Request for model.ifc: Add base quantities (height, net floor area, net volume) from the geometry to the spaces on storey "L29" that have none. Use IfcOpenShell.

First a look at what the model holds.

```python
import ifcopenshell
import ifcopenshell.util.element
import ifcopenshell.util.unit

model = ifcopenshell.open("model.ifc")
print(model.schema)
for unit_type in ("LENGTHUNIT", "AREAUNIT", "VOLUMEUNIT"):
    print(unit_type, ifcopenshell.util.unit.calculate_unit_scale(model, unit_type))
storey = next(s for s in model.by_type("IfcBuildingStorey") if s.Name == "L29")
spaces = [e for e in ifcopenshell.util.element.get_decomposition(storey) if e.is_a("IfcSpace")]
for e in sorted(spaces, key=lambda e: e.id()):
    print(e.id(), e.is_a(), e.Name, list(ifcopenshell.util.element.get_psets(e, qtos_only=True)), sep=" | ")
```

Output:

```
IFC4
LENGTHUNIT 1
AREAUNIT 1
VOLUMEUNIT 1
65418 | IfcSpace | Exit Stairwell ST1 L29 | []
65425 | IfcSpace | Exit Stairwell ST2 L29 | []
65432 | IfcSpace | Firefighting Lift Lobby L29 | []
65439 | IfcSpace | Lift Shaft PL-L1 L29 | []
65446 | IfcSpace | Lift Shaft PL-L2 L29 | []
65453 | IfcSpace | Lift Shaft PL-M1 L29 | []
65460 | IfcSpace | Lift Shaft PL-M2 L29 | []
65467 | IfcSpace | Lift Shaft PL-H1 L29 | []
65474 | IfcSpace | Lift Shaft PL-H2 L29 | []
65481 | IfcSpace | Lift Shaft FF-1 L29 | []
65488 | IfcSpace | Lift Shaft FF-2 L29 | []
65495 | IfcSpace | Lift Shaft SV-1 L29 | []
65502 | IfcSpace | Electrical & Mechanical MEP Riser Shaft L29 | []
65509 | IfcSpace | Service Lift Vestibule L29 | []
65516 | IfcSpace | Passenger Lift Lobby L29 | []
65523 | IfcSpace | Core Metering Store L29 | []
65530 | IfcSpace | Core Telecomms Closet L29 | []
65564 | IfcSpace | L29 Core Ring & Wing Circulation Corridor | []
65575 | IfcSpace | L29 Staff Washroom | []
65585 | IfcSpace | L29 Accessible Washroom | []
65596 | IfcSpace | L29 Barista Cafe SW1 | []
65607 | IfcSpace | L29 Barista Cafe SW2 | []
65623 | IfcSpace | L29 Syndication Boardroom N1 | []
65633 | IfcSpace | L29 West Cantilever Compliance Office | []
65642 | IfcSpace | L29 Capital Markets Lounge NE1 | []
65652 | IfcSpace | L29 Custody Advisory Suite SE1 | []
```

```python
import ifcopenshell
import ifcopenshell.api.pset
import ifcopenshell.geom
import ifcopenshell.util.element
import ifcopenshell.util.shape
import ifcopenshell.util.unit

model = ifcopenshell.open("model.ifc")
unit_scale = ifcopenshell.util.unit.calculate_unit_scale(model)
area_scale = ifcopenshell.util.unit.calculate_unit_scale(model, "AREAUNIT")
volume_scale = ifcopenshell.util.unit.calculate_unit_scale(model, "VOLUMEUNIT")
settings = ifcopenshell.geom.settings()

storey = next(s for s in model.by_type("IfcBuildingStorey") if s.Name == "L29")
spaces = [e for e in ifcopenshell.util.element.get_decomposition(storey) if e.is_a("IfcSpace")]

for e in sorted(spaces, key=lambda e: e.id()):
    if ifcopenshell.util.element.get_psets(e, qtos_only=True, should_inherit=False):
        continue
    # Geometry comes back in metres, in the element's own axes.
    shape = ifcopenshell.geom.create_shape(settings, e)
    values = {
        "Height": ifcopenshell.util.shape.get_z(shape.geometry) / unit_scale,
        "NetFloorArea": ifcopenshell.util.shape.get_footprint_area(shape.geometry) / area_scale,
        "NetVolume": ifcopenshell.util.shape.get_volume(shape.geometry) / volume_scale,
    }
    qto = ifcopenshell.api.pset.add_qto(model, product=e, name="Qto_SpaceBaseQuantities")
    ifcopenshell.api.pset.edit_qto(model, qto=qto, properties=values)
    print(e.id(), {k: round(v, 3) for k, v in values.items()})

model.write("model_v2.ifc")
```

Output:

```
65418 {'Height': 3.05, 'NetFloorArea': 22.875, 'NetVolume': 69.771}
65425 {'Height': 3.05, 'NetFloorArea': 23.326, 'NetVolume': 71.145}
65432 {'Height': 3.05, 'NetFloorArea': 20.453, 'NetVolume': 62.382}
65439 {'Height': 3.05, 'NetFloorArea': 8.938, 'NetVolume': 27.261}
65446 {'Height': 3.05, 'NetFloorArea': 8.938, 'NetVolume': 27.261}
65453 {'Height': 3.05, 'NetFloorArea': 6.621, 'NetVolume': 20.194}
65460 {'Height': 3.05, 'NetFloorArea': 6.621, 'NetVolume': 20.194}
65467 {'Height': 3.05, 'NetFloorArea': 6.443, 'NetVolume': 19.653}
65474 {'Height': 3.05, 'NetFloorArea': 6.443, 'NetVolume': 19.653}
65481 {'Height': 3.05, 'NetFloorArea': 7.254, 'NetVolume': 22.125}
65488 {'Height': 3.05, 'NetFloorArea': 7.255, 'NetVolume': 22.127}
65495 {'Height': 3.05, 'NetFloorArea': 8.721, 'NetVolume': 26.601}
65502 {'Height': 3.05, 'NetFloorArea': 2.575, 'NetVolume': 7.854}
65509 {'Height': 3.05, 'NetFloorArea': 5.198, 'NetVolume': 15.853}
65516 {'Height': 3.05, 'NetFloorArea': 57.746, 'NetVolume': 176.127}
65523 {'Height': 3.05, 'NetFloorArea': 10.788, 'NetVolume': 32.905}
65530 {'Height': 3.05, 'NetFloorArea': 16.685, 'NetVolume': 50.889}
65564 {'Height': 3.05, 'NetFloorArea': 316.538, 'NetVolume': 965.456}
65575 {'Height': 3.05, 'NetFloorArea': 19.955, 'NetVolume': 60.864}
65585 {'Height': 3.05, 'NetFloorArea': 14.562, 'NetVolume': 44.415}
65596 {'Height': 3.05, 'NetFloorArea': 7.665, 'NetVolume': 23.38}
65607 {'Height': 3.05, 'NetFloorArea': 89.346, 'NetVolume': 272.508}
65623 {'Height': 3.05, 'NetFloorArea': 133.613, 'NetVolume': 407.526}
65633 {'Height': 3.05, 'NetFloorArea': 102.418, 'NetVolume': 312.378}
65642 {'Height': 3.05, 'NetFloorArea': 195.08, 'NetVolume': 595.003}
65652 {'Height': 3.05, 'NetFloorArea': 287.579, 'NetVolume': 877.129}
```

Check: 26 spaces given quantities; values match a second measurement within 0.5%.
